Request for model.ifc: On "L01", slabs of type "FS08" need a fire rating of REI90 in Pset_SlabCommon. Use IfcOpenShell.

First a look at what the model holds.

```python
import ifcopenshell
import ifcopenshell.util.element

model = ifcopenshell.open("model.ifc")
print(model.schema)
storey = next(s for s in model.by_type("IfcBuildingStorey") if s.Name == "L01")
slabs = [e for e in ifcopenshell.util.element.get_decomposition(storey) if e.is_a("IfcSlab")]
seen = {}
for e in slabs:
    element_type = ifcopenshell.util.element.get_type(e)
    key = (element_type.Name if element_type != e and element_type else None, ifcopenshell.util.element.get_pset(e, "Pset_SlabCommon", "FireRating"))
    seen[key] = seen.get(key, 0) + 1
for (name, value), count in sorted(seen.items(), key=str):
    print(count, "x", name, "|", value)
```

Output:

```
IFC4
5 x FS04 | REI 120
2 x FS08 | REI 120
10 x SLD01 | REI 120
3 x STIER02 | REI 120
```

```python
import ifcopenshell
import ifcopenshell.api.pset
import ifcopenshell.util.element

model = ifcopenshell.open("model.ifc")

storey = next(s for s in model.by_type("IfcBuildingStorey") if s.Name == "L01")
slabs = [e for e in ifcopenshell.util.element.get_decomposition(storey) if e.is_a("IfcSlab")]

count = 0
for e in slabs:
    element_type = ifcopenshell.util.element.get_type(e)
    if element_type in (None, e) or element_type.Name != "FS08":
        continue
    # add_pset returns the element's existing set when there is one.
    pset = ifcopenshell.api.pset.add_pset(model, product=e, name="Pset_SlabCommon")
    ifcopenshell.api.pset.edit_pset(model, pset=pset, properties={"FireRating": "REI90"})
    count += 1

print(count, "slabs updated")

model.write("model_updated.ifc")
```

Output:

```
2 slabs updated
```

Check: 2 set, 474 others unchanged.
